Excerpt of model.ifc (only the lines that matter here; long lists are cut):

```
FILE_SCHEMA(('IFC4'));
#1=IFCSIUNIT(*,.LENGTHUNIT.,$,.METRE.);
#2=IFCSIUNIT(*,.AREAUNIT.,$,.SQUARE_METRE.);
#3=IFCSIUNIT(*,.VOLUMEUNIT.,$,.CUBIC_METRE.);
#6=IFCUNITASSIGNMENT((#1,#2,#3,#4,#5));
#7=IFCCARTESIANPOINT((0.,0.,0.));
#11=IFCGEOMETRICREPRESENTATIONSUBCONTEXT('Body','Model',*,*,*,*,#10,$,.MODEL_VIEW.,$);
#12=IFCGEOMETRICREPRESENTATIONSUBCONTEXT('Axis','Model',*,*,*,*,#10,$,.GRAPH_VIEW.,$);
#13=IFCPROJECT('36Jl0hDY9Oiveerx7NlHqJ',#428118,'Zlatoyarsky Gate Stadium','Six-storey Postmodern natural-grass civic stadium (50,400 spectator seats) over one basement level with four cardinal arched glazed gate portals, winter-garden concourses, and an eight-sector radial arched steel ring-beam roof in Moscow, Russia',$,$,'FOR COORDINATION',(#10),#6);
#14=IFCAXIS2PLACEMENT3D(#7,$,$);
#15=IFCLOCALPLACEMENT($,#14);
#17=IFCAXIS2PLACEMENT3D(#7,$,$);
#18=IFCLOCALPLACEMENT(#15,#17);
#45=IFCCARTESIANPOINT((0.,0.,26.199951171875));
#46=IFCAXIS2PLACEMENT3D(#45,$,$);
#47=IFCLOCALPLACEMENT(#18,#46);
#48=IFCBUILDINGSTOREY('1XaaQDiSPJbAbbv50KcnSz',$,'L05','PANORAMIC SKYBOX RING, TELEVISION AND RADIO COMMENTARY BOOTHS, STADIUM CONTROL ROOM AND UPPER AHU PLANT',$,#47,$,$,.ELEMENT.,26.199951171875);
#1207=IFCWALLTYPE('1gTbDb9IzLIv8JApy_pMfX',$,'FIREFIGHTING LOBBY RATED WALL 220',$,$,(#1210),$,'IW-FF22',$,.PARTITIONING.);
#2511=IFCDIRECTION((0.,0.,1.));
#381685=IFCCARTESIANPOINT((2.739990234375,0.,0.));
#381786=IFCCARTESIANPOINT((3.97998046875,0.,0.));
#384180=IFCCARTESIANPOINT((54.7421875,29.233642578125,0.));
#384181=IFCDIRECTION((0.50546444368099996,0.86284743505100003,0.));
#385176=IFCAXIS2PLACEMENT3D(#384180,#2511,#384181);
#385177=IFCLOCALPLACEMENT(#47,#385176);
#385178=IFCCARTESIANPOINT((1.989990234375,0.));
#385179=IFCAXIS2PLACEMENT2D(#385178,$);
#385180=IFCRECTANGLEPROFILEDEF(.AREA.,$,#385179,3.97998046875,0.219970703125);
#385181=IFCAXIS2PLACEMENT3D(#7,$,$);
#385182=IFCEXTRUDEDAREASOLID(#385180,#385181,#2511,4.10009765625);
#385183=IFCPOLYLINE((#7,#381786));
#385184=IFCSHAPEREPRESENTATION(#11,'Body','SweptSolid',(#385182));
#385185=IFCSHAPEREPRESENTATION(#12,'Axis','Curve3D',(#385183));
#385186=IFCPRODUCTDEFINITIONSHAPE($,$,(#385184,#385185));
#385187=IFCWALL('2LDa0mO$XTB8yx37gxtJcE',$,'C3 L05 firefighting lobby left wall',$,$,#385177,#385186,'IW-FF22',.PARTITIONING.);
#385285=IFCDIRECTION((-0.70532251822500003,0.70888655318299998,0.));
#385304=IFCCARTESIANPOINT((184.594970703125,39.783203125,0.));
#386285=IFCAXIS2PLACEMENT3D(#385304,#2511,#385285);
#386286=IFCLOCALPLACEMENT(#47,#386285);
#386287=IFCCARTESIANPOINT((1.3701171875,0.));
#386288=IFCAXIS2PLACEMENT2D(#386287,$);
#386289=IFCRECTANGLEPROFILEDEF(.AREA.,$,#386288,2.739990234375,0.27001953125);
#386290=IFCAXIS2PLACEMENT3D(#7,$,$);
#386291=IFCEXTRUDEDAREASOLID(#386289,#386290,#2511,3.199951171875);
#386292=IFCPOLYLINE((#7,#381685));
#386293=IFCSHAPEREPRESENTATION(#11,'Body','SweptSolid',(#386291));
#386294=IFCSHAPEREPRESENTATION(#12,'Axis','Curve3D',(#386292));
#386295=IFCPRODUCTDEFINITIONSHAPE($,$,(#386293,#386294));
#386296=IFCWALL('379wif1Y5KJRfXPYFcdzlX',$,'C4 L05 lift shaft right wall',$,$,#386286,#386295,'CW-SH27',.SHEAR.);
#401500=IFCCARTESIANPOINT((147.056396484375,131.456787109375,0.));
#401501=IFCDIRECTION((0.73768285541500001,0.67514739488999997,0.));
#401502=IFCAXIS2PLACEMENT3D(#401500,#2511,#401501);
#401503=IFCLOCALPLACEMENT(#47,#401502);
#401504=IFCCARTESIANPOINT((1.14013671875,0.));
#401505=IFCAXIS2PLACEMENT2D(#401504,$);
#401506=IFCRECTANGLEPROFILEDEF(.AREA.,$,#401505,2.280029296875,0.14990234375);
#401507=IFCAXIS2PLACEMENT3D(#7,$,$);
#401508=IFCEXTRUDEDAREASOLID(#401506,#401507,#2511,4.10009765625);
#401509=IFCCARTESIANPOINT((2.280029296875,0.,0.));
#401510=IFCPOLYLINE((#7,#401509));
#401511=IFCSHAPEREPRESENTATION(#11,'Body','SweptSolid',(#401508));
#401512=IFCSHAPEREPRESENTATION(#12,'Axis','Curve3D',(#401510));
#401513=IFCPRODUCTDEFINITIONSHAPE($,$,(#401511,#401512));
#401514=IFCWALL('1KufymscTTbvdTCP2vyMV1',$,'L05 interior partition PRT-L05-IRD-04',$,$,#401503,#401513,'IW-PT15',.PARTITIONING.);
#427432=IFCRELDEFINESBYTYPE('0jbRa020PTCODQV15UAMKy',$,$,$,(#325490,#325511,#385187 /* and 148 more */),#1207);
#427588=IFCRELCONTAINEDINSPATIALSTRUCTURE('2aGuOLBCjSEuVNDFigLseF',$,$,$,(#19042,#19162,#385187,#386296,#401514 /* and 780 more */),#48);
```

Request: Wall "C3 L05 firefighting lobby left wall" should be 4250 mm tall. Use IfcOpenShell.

```python
import ifcopenshell
import ifcopenshell.geom
import ifcopenshell.util.representation
import ifcopenshell.util.shape

model = ifcopenshell.open("model.ifc")
settings = ifcopenshell.geom.settings()


def volume(element):
    """Net volume in cubic metres, openings subtracted."""
    shape = ifcopenshell.geom.create_shape(settings, element)
    return ifcopenshell.util.shape.get_volume(shape.geometry)


wall = model.by_id(385187)
before = volume(wall)

body = ifcopenshell.util.representation.get_representation(wall, "Model", "Body")
solid = body.Items[0]
old_height = solid.Depth
solid.Depth = 4.25
after = volume(wall)

print(f"height {old_height:g} -> {solid.Depth:g}, volume {before:.3f} -> {after:.3f} m3")

model.write("model_rev.ifc")
```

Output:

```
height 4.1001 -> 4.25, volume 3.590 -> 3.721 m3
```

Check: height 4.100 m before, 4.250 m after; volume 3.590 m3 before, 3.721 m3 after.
